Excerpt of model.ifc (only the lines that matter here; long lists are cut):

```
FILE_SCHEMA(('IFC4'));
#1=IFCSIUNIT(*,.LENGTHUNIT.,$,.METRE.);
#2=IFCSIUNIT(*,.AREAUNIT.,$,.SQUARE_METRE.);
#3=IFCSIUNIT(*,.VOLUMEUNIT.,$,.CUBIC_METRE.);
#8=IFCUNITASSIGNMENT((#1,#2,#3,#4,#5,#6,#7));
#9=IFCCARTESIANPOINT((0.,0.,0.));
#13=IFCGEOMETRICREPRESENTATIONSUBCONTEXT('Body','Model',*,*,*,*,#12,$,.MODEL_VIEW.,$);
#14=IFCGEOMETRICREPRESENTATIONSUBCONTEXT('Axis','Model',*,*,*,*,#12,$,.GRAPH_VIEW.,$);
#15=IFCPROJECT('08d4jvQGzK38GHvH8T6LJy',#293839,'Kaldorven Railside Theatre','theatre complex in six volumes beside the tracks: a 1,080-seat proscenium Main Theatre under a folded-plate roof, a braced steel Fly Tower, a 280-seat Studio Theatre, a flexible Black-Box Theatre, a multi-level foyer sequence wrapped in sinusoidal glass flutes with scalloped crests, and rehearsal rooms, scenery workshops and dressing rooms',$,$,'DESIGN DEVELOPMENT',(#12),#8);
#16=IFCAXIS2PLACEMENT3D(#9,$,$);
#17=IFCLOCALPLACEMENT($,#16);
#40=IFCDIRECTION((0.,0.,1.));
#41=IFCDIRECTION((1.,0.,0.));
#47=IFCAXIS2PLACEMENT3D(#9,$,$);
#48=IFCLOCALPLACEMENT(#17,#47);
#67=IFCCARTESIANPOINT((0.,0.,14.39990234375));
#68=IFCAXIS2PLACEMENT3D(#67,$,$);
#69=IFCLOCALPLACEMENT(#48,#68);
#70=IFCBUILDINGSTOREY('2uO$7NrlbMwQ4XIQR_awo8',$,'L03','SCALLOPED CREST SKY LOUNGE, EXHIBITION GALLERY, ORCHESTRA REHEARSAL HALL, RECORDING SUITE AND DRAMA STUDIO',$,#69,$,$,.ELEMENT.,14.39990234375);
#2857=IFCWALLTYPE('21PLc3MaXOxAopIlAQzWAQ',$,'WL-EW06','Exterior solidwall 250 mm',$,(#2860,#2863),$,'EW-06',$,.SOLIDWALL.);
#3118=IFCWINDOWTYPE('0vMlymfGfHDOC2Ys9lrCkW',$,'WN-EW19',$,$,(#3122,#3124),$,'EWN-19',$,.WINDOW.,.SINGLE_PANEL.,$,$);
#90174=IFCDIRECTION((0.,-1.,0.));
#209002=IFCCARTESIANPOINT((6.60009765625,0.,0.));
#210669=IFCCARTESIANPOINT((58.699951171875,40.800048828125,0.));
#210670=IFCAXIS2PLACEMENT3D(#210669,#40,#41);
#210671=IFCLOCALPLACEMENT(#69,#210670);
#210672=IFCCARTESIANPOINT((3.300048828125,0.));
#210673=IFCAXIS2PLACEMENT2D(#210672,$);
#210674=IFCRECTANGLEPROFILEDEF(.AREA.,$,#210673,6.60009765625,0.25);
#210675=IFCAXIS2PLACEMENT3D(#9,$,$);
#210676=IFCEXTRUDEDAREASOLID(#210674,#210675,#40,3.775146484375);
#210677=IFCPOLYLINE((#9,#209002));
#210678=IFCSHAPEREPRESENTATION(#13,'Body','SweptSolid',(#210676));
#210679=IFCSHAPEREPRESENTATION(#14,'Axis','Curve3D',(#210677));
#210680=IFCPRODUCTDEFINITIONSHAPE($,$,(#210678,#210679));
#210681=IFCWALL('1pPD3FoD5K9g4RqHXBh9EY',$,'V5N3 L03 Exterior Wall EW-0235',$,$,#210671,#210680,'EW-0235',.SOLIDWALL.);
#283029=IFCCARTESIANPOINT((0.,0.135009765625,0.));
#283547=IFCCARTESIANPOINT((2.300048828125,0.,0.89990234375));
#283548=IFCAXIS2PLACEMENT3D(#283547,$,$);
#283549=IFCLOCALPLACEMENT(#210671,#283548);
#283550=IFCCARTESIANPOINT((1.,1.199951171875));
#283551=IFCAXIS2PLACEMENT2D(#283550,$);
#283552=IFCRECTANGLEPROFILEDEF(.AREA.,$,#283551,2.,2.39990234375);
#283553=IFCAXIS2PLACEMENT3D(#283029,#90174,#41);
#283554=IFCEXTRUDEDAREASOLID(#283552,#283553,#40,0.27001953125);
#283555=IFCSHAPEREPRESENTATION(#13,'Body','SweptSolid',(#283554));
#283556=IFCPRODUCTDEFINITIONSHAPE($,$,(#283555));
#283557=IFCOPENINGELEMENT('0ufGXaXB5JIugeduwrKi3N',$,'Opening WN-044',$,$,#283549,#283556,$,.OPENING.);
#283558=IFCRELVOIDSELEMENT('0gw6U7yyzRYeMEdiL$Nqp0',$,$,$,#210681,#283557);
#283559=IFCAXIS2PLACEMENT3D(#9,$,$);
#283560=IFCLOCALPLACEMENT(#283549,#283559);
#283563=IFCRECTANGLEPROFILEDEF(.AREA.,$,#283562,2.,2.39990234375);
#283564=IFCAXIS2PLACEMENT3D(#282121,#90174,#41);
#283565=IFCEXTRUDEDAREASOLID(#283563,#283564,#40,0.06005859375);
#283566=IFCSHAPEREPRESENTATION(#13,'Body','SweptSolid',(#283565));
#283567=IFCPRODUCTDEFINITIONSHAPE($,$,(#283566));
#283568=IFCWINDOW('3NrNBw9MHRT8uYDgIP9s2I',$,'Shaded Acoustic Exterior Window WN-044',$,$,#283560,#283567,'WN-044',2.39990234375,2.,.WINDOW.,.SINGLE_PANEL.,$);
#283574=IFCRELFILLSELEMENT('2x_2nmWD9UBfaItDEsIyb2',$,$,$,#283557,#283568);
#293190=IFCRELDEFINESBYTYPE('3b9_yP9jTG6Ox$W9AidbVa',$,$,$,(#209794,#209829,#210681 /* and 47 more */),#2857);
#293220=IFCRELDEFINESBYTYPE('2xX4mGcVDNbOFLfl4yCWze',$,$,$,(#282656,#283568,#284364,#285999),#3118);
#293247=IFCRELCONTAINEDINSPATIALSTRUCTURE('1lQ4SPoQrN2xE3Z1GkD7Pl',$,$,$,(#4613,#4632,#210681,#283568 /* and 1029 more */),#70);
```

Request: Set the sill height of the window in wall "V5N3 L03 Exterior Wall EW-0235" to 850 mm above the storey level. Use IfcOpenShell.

```python
import numpy as np
import ifcopenshell
import ifcopenshell.api.geometry
import ifcopenshell.geom
import ifcopenshell.util.element
import ifcopenshell.util.placement
import ifcopenshell.util.shape
import ifcopenshell.util.unit

model = ifcopenshell.open("model.ifc")
unit_scale = ifcopenshell.util.unit.calculate_unit_scale(model)

window = model.by_guid("3NrNBw9MHRT8uYDgIP9s2I")
opening = window.FillsVoids[0].RelatingOpeningElement
storey = ifcopenshell.util.element.get_container(window, ifc_class="IfcBuildingStorey")
level = ifcopenshell.util.placement.get_local_placement(storey.ObjectPlacement)[2, 3]

# The opening's origin need not be at the sill, so measure its lowest point.
shape = ifcopenshell.geom.create_shape(ifcopenshell.geom.settings(), opening)
bottom = ifcopenshell.util.shape.get_shape_bottom_elevation(shape, shape.geometry) / unit_scale
dz = level + 0.85 / unit_scale - bottom

shift = np.array([0.0, 0.0, dz])
# The window is placed relative to its opening, so it follows when the opening moves.
matrix = ifcopenshell.util.placement.get_local_placement(opening.ObjectPlacement)
matrix[:3, 3] += shift
ifcopenshell.api.geometry.edit_object_placement(
    model, product=opening, matrix=matrix, is_si=False, should_transform_children=True
)

print(f"moved by {dz * unit_scale:+.3f} m")

model.write("model_updated.ifc")
```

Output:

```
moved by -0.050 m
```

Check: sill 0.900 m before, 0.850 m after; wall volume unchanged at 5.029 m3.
